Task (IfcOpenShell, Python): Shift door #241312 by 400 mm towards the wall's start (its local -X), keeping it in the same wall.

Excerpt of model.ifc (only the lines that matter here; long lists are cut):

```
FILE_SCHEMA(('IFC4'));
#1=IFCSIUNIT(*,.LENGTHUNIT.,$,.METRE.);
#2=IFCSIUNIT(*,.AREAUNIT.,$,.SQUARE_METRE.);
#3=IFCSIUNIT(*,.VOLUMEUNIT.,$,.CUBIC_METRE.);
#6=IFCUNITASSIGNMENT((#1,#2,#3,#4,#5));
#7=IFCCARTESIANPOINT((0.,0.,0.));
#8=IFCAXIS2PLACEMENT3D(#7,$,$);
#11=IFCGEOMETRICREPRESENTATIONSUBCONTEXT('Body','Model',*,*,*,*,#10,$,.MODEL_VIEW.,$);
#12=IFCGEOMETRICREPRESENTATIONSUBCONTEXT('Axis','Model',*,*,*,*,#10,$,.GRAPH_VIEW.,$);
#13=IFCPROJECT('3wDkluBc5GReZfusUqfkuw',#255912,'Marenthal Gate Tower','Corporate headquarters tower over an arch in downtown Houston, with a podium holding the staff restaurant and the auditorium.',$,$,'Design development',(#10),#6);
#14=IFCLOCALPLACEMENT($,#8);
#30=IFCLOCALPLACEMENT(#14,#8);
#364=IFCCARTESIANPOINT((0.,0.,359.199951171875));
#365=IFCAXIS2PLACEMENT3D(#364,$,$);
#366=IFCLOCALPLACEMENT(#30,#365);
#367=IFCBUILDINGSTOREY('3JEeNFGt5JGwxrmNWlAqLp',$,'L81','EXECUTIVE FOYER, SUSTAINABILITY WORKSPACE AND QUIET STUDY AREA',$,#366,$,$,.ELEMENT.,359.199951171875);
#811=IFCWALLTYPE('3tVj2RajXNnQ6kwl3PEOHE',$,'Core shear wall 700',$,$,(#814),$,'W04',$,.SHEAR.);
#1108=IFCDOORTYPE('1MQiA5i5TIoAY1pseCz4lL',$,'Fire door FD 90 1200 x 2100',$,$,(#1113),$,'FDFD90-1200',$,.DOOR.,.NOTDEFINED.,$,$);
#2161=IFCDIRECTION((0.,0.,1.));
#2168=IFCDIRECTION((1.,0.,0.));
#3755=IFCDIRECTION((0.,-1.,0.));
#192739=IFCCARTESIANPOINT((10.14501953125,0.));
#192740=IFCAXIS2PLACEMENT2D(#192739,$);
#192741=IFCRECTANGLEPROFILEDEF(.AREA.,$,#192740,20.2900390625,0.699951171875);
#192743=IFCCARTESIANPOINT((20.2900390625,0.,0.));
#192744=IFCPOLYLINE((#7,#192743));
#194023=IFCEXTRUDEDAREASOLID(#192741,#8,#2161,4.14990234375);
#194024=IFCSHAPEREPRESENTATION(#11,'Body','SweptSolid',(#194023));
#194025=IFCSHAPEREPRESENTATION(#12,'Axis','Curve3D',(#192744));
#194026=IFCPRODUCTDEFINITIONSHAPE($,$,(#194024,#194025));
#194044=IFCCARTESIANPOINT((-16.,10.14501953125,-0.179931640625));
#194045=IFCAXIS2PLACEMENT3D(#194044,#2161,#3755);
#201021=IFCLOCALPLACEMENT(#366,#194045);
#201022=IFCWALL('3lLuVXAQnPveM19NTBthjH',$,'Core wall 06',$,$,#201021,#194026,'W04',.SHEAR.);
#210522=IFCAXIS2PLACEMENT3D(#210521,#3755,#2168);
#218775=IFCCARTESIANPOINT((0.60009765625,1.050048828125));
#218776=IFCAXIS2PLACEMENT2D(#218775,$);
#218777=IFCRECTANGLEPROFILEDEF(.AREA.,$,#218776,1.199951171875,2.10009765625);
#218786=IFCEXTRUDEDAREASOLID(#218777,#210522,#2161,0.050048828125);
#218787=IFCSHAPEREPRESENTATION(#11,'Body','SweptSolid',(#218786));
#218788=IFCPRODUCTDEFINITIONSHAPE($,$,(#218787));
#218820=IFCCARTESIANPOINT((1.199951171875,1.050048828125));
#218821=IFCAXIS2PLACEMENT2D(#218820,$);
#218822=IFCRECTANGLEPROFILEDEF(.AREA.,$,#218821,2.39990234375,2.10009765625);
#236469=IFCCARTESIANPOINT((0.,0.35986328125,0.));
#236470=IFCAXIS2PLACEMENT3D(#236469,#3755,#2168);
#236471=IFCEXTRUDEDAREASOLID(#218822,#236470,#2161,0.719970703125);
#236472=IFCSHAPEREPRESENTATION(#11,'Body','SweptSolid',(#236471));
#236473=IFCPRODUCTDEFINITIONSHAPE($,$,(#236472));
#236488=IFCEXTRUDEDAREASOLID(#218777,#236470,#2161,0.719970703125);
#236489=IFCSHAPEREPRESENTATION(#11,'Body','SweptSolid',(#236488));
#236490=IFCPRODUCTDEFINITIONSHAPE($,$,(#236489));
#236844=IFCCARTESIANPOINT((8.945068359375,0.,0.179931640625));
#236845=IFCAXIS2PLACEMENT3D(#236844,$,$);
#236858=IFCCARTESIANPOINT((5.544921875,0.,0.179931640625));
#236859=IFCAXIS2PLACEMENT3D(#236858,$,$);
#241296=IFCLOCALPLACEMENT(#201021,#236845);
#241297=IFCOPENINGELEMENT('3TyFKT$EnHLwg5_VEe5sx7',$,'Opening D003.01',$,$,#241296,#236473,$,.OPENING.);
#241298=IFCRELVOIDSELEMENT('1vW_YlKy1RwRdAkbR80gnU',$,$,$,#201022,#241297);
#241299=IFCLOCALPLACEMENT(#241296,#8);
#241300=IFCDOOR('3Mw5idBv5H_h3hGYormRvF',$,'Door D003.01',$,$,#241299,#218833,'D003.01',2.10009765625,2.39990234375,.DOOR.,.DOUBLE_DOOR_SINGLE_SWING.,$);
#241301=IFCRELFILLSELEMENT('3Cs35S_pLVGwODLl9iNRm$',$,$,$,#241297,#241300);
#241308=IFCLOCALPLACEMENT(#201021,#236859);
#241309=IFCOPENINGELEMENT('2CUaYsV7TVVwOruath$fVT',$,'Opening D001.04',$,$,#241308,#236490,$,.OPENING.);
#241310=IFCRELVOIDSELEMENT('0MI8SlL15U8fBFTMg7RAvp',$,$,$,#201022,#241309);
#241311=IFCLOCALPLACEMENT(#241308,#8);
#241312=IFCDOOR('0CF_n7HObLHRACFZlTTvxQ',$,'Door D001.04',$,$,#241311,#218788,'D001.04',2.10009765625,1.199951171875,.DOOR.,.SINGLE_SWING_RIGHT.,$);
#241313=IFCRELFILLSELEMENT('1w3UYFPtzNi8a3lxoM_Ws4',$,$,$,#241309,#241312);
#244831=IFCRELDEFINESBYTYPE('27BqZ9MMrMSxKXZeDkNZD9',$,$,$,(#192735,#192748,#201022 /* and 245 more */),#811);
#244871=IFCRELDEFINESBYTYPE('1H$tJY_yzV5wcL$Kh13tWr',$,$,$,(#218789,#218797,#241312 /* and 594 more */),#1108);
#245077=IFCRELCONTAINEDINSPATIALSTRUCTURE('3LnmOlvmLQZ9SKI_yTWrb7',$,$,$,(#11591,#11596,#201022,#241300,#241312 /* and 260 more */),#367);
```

```python
import ifcopenshell
import ifcopenshell.api.geometry
import ifcopenshell.util.placement
import ifcopenshell.util.unit

model = ifcopenshell.open("model.ifc")
unit_scale = ifcopenshell.util.unit.calculate_unit_scale(model)

door = model.by_id(241312)
opening = door.FillsVoids[0].RelatingOpeningElement
wall = opening.VoidsElements[0].RelatingBuildingElement

wall_matrix = ifcopenshell.util.placement.get_local_placement(wall.ObjectPlacement)
shift = wall_matrix[:3, 0] * -0.4 / unit_scale
before = ifcopenshell.util.placement.get_local_placement(door.ObjectPlacement)[:3, 3].copy()

# The door is placed relative to its opening, so it follows when the opening moves.
matrix = ifcopenshell.util.placement.get_local_placement(opening.ObjectPlacement)
matrix[:3, 3] += shift
ifcopenshell.api.geometry.edit_object_placement(
    model, product=opening, matrix=matrix, is_si=False, should_transform_children=True
)

after = ifcopenshell.util.placement.get_local_placement(door.ObjectPlacement)[:3, 3]
print("door moved by", (after - before).round(3) + 0.0)

model.write("model_v2.ifc")
```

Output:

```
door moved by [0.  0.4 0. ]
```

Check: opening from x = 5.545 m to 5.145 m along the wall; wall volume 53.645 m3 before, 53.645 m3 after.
